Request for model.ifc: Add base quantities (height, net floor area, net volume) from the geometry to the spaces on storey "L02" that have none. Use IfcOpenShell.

First a look at what the model holds.

```python
import ifcopenshell
import ifcopenshell.util.element
import ifcopenshell.util.unit

model = ifcopenshell.open("model.ifc")
print(model.schema)
for unit_type in ("LENGTHUNIT", "AREAUNIT", "VOLUMEUNIT"):
    print(unit_type, ifcopenshell.util.unit.calculate_unit_scale(model, unit_type))
storey = next(s for s in model.by_type("IfcBuildingStorey") if s.Name == "L02")
spaces = [e for e in ifcopenshell.util.element.get_decomposition(storey) if e.is_a("IfcSpace")]
for e in sorted(spaces, key=lambda e: e.id()):
    print(e.id(), e.is_a(), e.Name, list(ifcopenshell.util.element.get_psets(e, qtos_only=True)), sep=" | ")
```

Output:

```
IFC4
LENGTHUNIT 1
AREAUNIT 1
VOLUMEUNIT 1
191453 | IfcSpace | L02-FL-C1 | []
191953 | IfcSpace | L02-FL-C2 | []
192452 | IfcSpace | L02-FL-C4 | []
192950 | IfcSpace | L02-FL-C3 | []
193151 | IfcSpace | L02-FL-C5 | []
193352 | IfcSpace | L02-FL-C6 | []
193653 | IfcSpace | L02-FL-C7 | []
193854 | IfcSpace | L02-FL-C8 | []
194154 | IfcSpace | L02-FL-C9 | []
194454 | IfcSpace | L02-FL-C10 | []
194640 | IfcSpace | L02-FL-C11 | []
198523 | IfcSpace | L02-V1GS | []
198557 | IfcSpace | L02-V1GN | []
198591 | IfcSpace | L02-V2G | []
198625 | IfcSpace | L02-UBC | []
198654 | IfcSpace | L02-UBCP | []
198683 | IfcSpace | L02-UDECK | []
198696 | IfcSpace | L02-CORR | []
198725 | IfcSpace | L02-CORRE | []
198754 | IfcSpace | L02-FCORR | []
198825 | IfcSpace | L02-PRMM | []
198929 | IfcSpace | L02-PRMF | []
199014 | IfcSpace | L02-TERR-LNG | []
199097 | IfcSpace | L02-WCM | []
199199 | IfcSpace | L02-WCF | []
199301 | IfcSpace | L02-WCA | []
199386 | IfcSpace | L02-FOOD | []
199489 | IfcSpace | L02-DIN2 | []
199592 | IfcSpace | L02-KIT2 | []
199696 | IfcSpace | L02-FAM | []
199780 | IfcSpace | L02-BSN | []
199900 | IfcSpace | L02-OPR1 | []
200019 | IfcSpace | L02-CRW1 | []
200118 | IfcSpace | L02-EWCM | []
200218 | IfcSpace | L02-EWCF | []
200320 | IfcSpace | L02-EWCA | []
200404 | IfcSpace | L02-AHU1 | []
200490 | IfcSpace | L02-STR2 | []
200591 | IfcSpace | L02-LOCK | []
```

```python
import ifcopenshell
import ifcopenshell.api.pset
import ifcopenshell.geom
import ifcopenshell.util.element
import ifcopenshell.util.shape
import ifcopenshell.util.unit

model = ifcopenshell.open("model.ifc")
unit_scale = ifcopenshell.util.unit.calculate_unit_scale(model)
area_scale = ifcopenshell.util.unit.calculate_unit_scale(model, "AREAUNIT")
volume_scale = ifcopenshell.util.unit.calculate_unit_scale(model, "VOLUMEUNIT")
settings = ifcopenshell.geom.settings()

storey = next(s for s in model.by_type("IfcBuildingStorey") if s.Name == "L02")
spaces = [e for e in ifcopenshell.util.element.get_decomposition(storey) if e.is_a("IfcSpace")]

for e in sorted(spaces, key=lambda e: e.id()):
    if ifcopenshell.util.element.get_psets(e, qtos_only=True, should_inherit=False):
        continue
    # Geometry comes back in metres, in the element's own axes.
    shape = ifcopenshell.geom.create_shape(settings, e)
    values = {
        "Height": ifcopenshell.util.shape.get_z(shape.geometry) / unit_scale,
        "NetFloorArea": ifcopenshell.util.shape.get_footprint_area(shape.geometry) / area_scale,
        "NetVolume": ifcopenshell.util.shape.get_volume(shape.geometry) / volume_scale,
    }
    qto = ifcopenshell.api.pset.add_qto(model, product=e, name="Qto_SpaceBaseQuantities")
    ifcopenshell.api.pset.edit_qto(model, qto=qto, properties=values)
    print(e.id(), {k: round(v, 3) for k, v in values.items()})

model.write("model_v2.ifc")
```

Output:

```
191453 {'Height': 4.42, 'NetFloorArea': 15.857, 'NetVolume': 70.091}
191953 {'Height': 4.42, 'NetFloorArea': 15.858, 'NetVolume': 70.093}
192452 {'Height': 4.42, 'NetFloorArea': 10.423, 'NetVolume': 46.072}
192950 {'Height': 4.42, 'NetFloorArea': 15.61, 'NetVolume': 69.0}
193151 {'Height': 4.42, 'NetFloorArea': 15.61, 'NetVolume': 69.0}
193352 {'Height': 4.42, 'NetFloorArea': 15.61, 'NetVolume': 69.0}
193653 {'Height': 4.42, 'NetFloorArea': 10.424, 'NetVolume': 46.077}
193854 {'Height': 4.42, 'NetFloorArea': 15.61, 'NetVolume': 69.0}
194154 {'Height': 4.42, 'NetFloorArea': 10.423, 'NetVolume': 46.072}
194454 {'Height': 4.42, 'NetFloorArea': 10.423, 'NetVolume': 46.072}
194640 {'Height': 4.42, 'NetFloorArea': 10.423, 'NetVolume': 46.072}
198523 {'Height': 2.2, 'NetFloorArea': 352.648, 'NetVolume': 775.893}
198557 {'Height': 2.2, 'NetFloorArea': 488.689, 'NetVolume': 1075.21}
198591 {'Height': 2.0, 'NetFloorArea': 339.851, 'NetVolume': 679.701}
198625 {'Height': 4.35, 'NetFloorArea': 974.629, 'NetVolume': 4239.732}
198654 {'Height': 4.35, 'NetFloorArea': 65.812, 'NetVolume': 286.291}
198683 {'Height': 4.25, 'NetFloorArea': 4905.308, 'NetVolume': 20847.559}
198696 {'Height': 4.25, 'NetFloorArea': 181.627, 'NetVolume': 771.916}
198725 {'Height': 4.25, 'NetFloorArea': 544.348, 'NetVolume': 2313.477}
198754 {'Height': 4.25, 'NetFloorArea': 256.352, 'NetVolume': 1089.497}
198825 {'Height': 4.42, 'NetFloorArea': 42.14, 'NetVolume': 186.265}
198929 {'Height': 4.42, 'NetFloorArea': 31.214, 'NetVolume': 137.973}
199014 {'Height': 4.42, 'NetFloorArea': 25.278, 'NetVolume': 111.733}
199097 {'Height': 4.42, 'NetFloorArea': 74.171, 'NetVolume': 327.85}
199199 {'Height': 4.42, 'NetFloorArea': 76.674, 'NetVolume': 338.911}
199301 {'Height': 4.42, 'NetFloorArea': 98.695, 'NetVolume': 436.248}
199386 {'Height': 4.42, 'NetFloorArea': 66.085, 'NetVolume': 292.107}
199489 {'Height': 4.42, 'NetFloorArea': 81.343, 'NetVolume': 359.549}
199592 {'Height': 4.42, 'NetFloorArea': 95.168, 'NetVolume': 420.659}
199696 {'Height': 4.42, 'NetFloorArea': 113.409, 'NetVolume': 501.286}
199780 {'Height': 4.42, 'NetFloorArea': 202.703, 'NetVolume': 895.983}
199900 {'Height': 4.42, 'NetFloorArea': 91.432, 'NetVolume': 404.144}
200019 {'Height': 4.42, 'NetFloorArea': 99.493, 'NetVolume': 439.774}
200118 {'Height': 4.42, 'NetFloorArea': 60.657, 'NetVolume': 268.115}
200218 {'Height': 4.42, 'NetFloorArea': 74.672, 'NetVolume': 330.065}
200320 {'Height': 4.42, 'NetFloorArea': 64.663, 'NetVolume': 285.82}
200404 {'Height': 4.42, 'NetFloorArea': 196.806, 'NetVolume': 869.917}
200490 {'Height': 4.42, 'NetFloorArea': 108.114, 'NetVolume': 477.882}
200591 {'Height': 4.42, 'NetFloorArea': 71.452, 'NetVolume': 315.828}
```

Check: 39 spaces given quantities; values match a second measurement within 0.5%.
